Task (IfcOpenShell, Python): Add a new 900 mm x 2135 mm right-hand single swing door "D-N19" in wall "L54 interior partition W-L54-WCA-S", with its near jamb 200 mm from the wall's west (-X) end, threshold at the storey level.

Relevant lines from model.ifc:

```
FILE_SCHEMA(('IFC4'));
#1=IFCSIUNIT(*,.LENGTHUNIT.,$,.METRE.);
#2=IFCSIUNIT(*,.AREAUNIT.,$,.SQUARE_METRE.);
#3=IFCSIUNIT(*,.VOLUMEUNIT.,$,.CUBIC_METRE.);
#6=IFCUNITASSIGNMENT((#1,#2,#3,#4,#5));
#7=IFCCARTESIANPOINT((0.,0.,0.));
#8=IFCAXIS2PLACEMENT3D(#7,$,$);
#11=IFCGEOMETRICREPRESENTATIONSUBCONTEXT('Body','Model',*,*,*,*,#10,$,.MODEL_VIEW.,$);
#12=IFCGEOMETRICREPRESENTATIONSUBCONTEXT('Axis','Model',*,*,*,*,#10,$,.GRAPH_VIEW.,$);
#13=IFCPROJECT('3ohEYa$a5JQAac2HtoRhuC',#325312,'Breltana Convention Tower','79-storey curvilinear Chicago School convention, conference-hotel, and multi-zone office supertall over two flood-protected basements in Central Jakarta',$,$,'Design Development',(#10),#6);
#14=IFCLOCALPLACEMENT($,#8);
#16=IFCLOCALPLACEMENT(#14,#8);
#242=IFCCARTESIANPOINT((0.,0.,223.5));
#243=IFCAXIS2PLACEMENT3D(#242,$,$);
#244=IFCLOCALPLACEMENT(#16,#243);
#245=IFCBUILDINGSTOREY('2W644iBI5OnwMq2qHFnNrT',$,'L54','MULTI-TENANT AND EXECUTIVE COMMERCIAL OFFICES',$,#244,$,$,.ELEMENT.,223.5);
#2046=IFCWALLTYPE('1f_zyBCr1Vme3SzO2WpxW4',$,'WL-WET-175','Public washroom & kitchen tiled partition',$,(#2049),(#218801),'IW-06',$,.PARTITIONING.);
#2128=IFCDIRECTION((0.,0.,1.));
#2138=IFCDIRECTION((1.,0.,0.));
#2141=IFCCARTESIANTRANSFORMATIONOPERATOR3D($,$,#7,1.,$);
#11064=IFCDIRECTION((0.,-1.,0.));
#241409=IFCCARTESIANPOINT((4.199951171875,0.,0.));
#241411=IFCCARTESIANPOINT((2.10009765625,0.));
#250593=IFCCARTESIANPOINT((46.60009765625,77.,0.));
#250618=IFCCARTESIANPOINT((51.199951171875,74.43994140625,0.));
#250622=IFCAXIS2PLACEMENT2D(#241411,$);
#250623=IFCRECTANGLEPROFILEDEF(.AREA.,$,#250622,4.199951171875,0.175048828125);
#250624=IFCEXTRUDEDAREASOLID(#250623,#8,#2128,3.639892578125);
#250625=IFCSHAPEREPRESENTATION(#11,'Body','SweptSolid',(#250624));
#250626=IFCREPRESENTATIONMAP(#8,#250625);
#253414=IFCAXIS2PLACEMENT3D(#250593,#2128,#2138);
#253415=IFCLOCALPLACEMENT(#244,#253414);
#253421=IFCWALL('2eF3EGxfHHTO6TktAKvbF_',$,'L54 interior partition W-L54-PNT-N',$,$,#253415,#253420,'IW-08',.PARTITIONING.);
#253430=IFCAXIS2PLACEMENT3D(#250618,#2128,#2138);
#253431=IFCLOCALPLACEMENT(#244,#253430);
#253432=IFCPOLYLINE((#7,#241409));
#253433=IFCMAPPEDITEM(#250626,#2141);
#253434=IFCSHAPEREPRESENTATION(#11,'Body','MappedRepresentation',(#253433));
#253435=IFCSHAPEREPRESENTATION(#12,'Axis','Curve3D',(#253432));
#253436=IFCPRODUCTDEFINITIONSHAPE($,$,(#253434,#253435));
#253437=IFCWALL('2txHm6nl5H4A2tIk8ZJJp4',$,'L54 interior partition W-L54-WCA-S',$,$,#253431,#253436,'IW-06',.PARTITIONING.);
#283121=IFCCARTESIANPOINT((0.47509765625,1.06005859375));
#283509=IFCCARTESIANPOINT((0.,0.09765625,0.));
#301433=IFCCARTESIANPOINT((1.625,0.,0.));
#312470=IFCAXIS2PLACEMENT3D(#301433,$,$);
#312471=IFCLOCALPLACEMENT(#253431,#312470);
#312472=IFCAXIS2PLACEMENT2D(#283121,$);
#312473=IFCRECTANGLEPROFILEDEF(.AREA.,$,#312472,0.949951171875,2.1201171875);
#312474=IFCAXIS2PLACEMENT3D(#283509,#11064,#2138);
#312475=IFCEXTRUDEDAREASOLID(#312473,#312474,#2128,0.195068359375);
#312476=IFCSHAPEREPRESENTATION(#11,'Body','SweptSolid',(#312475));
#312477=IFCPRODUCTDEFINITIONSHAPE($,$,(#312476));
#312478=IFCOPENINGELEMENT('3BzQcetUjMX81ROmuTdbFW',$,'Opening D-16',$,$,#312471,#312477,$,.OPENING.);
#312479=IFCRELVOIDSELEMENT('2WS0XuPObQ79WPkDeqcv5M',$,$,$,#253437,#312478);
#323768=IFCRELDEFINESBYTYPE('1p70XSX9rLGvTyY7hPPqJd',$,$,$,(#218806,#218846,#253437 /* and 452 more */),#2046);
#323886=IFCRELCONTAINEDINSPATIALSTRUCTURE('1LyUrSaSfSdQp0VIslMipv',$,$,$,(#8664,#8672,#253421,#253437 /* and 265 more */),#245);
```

```python
import numpy as np
import ifcopenshell
import ifcopenshell.api.feature
import ifcopenshell.api.geometry
import ifcopenshell.api.root
import ifcopenshell.api.spatial
import ifcopenshell.geom
import ifcopenshell.util.element
import ifcopenshell.util.placement
import ifcopenshell.util.representation
import ifcopenshell.util.shape
import ifcopenshell.util.unit

model = ifcopenshell.open("model.ifc")
unit_scale = ifcopenshell.util.unit.calculate_unit_scale(model)
settings = ifcopenshell.geom.settings()


def volume(element):
    """Net volume in cubic metres, openings subtracted."""
    shape = ifcopenshell.geom.create_shape(settings, element)
    return ifcopenshell.util.shape.get_volume(shape.geometry)


wall = model.by_guid("2txHm6nl5H4A2tIk8ZJJp4")
storey = ifcopenshell.util.element.get_container(wall, ifc_class="IfcBuildingStorey")
context = ifcopenshell.util.representation.get_context(model, "Model", "Body", "MODEL_VIEW")
before = volume(wall)

width, height, from_end, sill = 0.9, 2.135, 0.2, 0.0  # metres

# The wall runs along its own X axis, and the end named is its -X end.
wall_shape = ifcopenshell.geom.create_shape(settings, wall)
x, y, z = ifcopenshell.util.shape.get_vertices(wall_shape.geometry).T
start = x.min() + from_end
face, thickness = float(y.min()), float(y.max() - y.min())
wall_matrix = ifcopenshell.util.placement.get_local_placement(wall.ObjectPlacement)
level = ifcopenshell.util.placement.get_local_placement(storey.ObjectPlacement)[2, 3]


def in_wall(x, y):
    """Placement at x, y metres in the wall's axes, at sill height."""
    matrix = wall_matrix.copy()
    matrix[:, 3] = wall_matrix @ np.array([x / unit_scale, y / unit_scale, 0.0, 1.0])
    matrix[2, 3] = level + sill / unit_scale
    return matrix


# Opening: a box that overshoots both wall faces by 50 mm.
opening = ifcopenshell.api.root.create_entity(model, ifc_class="IfcOpeningElement", predefined_type="OPENING")
box = ifcopenshell.api.geometry.add_wall_representation(
    model, context=context, length=width, height=height, thickness=thickness + 0.1
)
ifcopenshell.api.geometry.assign_representation(model, product=opening, representation=box)
ifcopenshell.api.geometry.edit_object_placement(model, product=opening, matrix=in_wall(start, face - 0.05), is_si=False)
ifcopenshell.api.feature.add_feature(model, feature=opening, element=wall)

door = ifcopenshell.api.root.create_entity(model, ifc_class="IfcDoor", name="D-N19", predefined_type="DOOR")
door.OverallWidth, door.OverallHeight = width / unit_scale, height / unit_scale
door.OperationType = "SINGLE_SWING_RIGHT"
body = ifcopenshell.api.geometry.add_door_representation(
    model,
    context=context,
    overall_width=door.OverallWidth,
    overall_height=door.OverallHeight,
    operation_type="SINGLE_SWING_RIGHT",
    lining_properties={"LiningDepth": thickness / unit_scale, "ThresholdDepth": thickness / unit_scale},
)
ifcopenshell.api.geometry.assign_representation(model, product=door, representation=body)
ifcopenshell.api.spatial.assign_container(model, products=[door], relating_structure=storey)
ifcopenshell.api.feature.add_filling(model, opening=opening, element=door)

# The lining spans the wall, so the door starts at the wall face.
ifcopenshell.api.geometry.edit_object_placement(model, product=door, matrix=in_wall(start, face), is_si=False)

after = volume(wall)

print(f"wall volume {before:.3f} -> {after:.3f} m3")

model.write("model_rev.ifc")
```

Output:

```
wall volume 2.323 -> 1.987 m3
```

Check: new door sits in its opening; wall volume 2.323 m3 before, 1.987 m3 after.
